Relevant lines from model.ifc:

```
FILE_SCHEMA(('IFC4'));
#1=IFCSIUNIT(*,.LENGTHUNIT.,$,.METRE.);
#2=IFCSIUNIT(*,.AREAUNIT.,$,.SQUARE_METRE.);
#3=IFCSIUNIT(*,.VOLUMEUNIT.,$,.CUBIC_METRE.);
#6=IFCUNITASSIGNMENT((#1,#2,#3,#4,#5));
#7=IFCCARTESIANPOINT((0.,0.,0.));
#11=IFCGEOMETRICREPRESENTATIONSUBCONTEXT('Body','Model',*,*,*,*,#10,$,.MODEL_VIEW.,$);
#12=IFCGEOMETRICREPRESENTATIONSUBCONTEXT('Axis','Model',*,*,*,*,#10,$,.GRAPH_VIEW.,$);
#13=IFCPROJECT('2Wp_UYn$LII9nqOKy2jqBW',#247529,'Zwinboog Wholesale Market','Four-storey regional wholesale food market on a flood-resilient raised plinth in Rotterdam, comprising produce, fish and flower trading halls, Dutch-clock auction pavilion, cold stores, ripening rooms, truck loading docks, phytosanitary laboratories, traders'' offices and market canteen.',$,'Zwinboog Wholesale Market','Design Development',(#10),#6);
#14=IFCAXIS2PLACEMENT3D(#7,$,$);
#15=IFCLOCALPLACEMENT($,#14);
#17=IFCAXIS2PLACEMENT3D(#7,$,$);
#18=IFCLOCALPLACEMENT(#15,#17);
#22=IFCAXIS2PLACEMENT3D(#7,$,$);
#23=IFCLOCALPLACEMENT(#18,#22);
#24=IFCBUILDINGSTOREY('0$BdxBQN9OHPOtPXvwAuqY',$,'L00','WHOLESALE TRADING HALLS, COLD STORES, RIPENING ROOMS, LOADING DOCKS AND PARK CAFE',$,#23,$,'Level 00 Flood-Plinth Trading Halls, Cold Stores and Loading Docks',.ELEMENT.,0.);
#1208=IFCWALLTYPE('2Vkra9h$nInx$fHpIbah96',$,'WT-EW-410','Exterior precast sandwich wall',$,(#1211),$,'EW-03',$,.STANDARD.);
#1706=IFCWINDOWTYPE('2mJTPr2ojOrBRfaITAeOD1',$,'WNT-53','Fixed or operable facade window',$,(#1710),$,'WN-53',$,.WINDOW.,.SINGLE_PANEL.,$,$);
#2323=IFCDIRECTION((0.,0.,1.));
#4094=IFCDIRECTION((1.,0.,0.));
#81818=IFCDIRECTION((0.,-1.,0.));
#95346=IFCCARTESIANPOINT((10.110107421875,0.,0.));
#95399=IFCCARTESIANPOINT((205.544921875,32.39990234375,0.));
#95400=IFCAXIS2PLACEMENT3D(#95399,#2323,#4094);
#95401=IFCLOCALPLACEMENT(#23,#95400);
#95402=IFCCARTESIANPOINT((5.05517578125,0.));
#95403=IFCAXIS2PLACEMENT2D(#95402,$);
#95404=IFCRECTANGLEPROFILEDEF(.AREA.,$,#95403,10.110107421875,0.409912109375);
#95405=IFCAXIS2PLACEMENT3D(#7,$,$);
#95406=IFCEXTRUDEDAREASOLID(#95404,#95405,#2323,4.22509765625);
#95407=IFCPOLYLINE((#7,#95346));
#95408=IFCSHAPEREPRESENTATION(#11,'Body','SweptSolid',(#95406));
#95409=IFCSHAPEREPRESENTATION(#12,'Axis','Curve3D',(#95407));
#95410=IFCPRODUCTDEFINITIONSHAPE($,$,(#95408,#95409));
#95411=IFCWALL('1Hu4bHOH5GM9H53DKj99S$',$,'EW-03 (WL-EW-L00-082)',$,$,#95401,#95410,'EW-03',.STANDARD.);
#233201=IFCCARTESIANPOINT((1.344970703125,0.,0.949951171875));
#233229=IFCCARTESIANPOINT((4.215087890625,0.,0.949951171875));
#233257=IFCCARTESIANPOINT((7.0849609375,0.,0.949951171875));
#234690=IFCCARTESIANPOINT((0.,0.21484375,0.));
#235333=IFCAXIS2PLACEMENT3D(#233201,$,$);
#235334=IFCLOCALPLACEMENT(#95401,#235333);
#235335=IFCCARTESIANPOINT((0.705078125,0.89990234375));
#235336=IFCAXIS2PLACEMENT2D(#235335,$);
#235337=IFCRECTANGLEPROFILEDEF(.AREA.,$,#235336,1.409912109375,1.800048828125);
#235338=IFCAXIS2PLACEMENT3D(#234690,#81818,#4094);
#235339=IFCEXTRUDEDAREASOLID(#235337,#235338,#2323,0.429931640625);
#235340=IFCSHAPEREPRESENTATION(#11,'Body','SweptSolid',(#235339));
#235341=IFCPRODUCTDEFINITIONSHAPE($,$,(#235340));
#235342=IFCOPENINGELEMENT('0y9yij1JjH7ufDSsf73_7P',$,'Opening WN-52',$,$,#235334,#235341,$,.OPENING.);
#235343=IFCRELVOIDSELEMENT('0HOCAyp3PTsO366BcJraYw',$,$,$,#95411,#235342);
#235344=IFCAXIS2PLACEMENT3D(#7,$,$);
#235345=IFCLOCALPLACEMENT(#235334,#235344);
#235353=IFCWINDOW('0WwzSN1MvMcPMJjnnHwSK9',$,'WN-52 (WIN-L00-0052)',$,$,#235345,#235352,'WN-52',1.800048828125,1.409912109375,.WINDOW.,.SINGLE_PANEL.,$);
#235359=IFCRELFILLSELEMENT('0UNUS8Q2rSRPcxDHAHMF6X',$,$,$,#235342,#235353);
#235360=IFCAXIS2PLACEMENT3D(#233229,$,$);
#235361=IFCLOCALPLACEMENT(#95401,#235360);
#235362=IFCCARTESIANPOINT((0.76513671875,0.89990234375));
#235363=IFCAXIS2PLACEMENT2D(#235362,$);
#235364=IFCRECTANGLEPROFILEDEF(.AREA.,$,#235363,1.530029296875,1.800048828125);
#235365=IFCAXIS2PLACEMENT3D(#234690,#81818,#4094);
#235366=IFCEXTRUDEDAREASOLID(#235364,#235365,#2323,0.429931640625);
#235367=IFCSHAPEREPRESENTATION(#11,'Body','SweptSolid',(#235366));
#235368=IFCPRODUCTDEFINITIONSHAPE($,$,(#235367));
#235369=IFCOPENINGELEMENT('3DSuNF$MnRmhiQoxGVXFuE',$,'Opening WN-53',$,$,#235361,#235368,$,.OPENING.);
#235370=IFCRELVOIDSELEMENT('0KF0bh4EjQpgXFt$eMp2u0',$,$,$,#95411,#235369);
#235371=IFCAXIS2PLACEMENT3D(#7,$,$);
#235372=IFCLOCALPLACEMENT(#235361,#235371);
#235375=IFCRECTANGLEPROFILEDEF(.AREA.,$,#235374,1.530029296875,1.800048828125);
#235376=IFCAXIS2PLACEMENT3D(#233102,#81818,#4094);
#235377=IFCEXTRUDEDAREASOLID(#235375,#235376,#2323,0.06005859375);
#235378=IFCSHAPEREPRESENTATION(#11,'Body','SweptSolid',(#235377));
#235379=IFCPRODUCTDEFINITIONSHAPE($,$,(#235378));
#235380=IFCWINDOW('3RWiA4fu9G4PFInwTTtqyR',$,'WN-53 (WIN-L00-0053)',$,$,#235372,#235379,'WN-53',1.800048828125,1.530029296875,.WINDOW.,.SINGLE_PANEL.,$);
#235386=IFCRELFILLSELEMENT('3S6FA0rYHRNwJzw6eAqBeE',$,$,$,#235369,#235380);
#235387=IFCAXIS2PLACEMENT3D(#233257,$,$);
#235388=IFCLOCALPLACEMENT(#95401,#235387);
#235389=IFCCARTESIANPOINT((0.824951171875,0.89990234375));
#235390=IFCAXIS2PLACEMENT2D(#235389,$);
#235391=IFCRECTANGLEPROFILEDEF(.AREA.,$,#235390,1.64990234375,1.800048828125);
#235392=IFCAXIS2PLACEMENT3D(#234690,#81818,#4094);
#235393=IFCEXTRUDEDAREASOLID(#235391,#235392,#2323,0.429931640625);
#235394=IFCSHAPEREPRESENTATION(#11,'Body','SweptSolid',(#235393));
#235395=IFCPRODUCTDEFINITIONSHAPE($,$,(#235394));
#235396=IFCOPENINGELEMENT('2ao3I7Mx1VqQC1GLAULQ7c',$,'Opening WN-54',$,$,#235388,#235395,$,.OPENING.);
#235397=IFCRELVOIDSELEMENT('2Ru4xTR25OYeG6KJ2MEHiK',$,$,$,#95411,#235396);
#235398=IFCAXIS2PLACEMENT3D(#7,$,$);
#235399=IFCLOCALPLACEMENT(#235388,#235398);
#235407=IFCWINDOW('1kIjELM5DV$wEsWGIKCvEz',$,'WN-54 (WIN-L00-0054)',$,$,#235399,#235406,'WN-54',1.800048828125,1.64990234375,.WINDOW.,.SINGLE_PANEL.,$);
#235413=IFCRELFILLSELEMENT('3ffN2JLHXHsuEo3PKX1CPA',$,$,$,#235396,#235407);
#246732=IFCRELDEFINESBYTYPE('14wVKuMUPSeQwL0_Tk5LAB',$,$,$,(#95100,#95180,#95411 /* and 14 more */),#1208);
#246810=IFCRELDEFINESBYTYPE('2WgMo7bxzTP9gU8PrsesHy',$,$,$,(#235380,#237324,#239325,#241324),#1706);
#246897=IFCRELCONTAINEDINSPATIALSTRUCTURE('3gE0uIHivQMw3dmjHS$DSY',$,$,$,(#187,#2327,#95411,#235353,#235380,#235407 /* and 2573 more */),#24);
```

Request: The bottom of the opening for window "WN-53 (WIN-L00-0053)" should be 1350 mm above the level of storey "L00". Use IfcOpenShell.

```python
import numpy as np
import ifcopenshell
import ifcopenshell.api.geometry
import ifcopenshell.geom
import ifcopenshell.util.element
import ifcopenshell.util.placement
import ifcopenshell.util.shape
import ifcopenshell.util.unit

model = ifcopenshell.open("model.ifc")
unit_scale = ifcopenshell.util.unit.calculate_unit_scale(model)

window = model.by_id(235380)
opening = window.FillsVoids[0].RelatingOpeningElement
storey = ifcopenshell.util.element.get_container(window, ifc_class="IfcBuildingStorey")
level = ifcopenshell.util.placement.get_local_placement(storey.ObjectPlacement)[2, 3]

# The opening's origin need not be at the sill, so measure its lowest point.
shape = ifcopenshell.geom.create_shape(ifcopenshell.geom.settings(), opening)
bottom = ifcopenshell.util.shape.get_shape_bottom_elevation(shape, shape.geometry) / unit_scale
dz = level + 1.35 / unit_scale - bottom

shift = np.array([0.0, 0.0, dz])
# The window is placed relative to its opening, so it follows when the opening moves.
matrix = ifcopenshell.util.placement.get_local_placement(opening.ObjectPlacement)
matrix[:3, 3] += shift
ifcopenshell.api.geometry.edit_object_placement(
    model, product=opening, matrix=matrix, is_si=False, should_transform_children=True
)

print(f"moved by {dz * unit_scale:+.3f} m")

model.write("model-out.ifc")
```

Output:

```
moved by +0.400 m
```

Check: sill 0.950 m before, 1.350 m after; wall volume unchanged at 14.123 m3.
